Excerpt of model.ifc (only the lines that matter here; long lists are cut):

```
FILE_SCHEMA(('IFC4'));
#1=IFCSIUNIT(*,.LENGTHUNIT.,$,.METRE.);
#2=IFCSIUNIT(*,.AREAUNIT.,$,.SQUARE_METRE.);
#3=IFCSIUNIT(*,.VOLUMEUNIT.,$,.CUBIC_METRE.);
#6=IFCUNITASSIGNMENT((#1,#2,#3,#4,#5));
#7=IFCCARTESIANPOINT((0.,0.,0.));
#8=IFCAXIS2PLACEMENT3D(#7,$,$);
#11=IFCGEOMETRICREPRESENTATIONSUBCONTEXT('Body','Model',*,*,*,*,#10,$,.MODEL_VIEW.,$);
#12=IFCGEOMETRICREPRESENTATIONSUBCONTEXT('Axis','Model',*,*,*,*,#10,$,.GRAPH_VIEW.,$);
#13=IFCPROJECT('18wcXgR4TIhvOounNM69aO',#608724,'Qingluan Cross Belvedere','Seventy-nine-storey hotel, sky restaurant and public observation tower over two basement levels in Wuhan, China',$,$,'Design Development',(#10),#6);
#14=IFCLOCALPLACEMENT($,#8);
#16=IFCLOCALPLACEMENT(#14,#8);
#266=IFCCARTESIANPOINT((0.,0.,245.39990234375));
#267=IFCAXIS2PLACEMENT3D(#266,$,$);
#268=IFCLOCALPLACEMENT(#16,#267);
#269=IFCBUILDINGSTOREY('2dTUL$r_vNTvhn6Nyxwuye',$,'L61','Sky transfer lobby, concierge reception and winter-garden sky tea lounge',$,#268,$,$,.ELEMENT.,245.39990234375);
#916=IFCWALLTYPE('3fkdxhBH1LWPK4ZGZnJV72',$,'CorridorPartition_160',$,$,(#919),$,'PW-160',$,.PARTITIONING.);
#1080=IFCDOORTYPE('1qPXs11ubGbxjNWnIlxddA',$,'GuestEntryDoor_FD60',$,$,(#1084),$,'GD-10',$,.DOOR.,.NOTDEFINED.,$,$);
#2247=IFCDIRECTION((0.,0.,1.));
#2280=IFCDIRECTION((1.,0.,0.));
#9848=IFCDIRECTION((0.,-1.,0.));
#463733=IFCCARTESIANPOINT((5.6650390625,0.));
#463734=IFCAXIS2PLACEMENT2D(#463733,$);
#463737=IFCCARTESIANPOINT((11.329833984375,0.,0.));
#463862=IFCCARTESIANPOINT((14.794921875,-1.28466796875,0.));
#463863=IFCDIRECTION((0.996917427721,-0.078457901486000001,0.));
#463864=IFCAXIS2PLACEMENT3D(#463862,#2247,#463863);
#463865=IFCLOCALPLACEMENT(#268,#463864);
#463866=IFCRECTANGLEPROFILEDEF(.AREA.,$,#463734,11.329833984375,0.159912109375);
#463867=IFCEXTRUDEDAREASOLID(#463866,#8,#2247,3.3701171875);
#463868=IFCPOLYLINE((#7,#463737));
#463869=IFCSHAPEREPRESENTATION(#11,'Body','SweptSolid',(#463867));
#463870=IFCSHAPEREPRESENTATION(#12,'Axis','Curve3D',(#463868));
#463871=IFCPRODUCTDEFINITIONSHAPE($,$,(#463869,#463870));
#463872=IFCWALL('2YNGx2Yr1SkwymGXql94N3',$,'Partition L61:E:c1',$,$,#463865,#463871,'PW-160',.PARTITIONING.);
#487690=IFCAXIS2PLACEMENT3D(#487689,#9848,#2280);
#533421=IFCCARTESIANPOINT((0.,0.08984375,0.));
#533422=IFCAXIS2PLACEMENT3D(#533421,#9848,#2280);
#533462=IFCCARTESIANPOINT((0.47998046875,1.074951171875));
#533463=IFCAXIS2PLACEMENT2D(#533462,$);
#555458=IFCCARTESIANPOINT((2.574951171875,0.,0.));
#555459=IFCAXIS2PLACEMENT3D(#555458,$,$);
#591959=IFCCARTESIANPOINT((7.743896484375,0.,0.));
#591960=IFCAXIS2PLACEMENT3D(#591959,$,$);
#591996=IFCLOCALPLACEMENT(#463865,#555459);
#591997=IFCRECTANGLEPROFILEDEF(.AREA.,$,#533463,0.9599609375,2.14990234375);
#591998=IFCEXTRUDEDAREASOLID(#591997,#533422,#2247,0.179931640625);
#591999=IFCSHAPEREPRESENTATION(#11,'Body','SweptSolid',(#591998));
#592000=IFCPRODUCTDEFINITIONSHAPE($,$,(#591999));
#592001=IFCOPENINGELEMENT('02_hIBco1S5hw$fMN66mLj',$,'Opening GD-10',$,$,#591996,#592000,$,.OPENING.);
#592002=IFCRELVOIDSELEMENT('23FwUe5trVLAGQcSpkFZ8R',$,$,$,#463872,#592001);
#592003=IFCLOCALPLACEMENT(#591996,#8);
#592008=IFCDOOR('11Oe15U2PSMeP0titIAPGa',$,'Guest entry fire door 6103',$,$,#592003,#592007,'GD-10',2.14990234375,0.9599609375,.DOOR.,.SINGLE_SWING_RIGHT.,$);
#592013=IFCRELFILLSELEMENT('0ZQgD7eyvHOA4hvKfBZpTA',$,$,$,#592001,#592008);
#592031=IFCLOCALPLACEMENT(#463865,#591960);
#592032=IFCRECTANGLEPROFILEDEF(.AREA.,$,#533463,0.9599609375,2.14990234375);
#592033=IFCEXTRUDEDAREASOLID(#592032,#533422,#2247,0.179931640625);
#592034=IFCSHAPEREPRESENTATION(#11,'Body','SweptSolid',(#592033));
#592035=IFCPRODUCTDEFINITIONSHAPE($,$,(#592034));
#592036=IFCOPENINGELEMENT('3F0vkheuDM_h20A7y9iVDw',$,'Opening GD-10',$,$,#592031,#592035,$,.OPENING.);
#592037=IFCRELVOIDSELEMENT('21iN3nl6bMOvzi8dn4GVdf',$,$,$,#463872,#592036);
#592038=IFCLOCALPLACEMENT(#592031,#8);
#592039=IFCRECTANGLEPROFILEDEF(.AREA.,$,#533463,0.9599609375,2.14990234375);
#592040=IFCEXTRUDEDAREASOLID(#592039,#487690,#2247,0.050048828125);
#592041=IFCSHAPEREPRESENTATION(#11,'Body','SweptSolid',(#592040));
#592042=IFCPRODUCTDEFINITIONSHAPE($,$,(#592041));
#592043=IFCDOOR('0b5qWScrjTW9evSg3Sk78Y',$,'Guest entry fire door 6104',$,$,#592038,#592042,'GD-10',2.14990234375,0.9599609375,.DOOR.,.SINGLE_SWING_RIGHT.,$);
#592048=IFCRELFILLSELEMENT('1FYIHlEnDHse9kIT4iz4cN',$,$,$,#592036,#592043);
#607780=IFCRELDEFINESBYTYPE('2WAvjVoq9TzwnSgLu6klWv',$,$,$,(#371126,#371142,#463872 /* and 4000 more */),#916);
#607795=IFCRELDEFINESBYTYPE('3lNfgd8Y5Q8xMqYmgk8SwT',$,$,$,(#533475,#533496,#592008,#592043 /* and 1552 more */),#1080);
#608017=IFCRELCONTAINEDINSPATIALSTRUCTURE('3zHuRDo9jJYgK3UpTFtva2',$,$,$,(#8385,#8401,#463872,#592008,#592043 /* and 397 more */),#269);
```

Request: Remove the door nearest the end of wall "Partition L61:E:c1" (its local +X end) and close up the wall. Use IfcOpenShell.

```python
import ifcopenshell
import ifcopenshell.api.feature
import ifcopenshell.api.root
import ifcopenshell.geom
import ifcopenshell.util.shape

model = ifcopenshell.open("model.ifc")
settings = ifcopenshell.geom.settings()


def volume(element):
    """Net volume in cubic metres, openings subtracted."""
    shape = ifcopenshell.geom.create_shape(settings, element)
    return ifcopenshell.util.shape.get_volume(shape.geometry)


door = model.by_guid("0b5qWScrjTW9evSg3Sk78Y")
opening = door.FillsVoids[0].RelatingOpeningElement
wall = opening.VoidsElements[0].RelatingBuildingElement
before = volume(wall)

ifcopenshell.api.root.remove_product(model, product=door)
ifcopenshell.api.feature.remove_feature(model, feature=opening)

after = volume(wall)

print(f"wall volume {before:.3f} -> {after:.3f} m3")

model.write("model-out.ifc")
```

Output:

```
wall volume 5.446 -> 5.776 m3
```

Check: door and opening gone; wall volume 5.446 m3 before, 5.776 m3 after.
